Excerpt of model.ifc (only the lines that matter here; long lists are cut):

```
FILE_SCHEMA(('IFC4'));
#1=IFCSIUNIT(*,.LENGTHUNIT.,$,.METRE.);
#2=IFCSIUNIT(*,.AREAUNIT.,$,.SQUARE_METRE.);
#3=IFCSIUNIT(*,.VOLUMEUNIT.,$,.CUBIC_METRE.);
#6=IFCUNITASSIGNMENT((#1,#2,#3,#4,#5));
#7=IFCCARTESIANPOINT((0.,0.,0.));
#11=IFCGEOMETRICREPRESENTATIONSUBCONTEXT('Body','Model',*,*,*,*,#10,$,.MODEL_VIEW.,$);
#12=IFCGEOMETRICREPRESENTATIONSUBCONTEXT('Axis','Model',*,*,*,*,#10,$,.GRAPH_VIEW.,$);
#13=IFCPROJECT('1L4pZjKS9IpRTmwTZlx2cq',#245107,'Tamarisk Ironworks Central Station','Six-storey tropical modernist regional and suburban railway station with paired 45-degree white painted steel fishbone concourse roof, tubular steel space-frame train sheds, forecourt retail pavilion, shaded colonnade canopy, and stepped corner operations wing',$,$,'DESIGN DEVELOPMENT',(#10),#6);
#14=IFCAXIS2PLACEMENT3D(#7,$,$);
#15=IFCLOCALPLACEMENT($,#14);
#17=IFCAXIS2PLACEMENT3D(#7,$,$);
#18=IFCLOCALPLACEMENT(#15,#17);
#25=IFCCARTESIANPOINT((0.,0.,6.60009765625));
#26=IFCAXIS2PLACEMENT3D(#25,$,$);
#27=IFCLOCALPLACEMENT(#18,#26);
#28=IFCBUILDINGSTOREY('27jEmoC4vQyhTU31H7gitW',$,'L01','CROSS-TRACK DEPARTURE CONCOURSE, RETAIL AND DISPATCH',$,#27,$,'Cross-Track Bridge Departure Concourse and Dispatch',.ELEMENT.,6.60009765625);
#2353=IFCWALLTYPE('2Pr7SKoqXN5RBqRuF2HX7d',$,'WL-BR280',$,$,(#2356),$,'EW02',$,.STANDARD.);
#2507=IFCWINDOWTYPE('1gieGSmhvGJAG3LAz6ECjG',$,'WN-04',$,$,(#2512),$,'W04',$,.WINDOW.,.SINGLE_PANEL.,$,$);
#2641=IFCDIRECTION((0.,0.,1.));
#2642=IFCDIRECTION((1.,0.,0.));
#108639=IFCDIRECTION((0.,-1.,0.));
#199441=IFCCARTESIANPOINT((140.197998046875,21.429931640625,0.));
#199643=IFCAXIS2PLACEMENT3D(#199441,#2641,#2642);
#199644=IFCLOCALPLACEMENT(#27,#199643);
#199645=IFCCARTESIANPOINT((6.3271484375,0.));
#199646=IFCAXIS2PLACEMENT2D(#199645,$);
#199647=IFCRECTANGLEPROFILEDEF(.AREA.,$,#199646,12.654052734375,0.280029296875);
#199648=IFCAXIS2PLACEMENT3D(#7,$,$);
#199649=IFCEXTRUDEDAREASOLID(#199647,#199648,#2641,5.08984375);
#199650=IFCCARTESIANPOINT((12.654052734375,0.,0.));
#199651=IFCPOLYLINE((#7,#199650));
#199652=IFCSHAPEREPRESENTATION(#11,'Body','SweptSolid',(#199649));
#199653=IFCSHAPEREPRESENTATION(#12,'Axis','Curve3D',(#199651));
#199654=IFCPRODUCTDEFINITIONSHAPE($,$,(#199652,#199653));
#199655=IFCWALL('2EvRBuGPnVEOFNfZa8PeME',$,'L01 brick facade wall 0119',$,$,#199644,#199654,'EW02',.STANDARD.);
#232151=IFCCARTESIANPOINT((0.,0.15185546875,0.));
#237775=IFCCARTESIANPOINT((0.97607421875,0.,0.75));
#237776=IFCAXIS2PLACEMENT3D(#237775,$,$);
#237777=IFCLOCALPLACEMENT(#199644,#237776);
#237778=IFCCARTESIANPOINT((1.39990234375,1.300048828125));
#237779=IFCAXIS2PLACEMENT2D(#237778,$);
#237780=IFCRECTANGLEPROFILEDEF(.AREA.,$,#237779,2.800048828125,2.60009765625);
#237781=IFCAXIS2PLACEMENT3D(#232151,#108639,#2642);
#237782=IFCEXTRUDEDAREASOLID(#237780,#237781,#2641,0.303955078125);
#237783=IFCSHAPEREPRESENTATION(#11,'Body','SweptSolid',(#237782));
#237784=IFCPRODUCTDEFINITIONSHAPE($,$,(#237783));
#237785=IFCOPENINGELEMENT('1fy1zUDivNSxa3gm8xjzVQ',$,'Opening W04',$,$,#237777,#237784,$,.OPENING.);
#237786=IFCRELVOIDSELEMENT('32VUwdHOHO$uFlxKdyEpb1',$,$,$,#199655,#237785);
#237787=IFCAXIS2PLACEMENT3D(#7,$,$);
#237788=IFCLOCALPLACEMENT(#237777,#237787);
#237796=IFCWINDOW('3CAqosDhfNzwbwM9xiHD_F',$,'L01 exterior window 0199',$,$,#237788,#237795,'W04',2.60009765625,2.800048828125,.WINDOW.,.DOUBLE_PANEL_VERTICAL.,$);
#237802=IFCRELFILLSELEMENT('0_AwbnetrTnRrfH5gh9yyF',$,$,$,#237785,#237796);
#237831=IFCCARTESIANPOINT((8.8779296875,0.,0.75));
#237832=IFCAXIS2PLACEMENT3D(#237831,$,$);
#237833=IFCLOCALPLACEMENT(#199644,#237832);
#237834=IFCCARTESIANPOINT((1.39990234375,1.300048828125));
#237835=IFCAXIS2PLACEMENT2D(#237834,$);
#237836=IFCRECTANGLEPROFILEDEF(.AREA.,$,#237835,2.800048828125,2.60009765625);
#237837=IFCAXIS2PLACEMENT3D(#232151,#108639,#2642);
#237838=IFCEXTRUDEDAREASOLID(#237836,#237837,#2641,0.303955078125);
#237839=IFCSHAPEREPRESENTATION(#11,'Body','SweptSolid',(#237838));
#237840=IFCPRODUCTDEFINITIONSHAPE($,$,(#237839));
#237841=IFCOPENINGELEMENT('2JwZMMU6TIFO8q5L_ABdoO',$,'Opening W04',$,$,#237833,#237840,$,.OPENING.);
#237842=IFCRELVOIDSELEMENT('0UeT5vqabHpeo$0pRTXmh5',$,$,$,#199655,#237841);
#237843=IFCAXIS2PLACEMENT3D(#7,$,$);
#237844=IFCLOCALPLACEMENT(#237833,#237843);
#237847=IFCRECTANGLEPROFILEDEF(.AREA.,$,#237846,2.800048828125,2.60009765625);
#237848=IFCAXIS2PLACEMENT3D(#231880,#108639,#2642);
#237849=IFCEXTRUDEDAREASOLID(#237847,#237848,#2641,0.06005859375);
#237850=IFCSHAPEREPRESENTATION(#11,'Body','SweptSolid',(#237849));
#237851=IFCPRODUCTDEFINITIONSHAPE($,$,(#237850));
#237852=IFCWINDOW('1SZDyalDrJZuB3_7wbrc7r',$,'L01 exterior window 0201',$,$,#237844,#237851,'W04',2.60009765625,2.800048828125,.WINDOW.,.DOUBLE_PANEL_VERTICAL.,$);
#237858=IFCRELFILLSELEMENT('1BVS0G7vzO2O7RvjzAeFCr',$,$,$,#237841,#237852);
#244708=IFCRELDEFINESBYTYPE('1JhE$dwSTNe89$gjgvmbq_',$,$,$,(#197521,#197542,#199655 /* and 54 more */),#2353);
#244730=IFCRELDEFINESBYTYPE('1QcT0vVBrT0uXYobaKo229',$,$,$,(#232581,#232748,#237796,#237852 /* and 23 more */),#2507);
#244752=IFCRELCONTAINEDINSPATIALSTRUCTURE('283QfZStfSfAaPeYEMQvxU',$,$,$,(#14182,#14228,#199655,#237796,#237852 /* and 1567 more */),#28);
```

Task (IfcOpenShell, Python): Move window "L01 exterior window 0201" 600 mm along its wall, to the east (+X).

```python
import ifcopenshell
import ifcopenshell.api.geometry
import ifcopenshell.util.placement

model = ifcopenshell.open("model.ifc")

window = model.by_guid("1SZDyalDrJZuB3_7wbrc7r")
opening = window.FillsVoids[0].RelatingOpeningElement
wall = opening.VoidsElements[0].RelatingBuildingElement

wall_matrix = ifcopenshell.util.placement.get_local_placement(wall.ObjectPlacement)
shift = wall_matrix[:3, 0] * 0.6
before = ifcopenshell.util.placement.get_local_placement(window.ObjectPlacement)[:3, 3].copy()

# The window is placed relative to its opening, so it follows when the opening moves.
matrix = ifcopenshell.util.placement.get_local_placement(opening.ObjectPlacement)
matrix[:3, 3] += shift
ifcopenshell.api.geometry.edit_object_placement(
    model, product=opening, matrix=matrix, is_si=False, should_transform_children=True
)

after = ifcopenshell.util.placement.get_local_placement(window.ObjectPlacement)[:3, 3]
print("window moved by", (after - before).round(3) + 0.0)

model.write("model_edited.ifc")
```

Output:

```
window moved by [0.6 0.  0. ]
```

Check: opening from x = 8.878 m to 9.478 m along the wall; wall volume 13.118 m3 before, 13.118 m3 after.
